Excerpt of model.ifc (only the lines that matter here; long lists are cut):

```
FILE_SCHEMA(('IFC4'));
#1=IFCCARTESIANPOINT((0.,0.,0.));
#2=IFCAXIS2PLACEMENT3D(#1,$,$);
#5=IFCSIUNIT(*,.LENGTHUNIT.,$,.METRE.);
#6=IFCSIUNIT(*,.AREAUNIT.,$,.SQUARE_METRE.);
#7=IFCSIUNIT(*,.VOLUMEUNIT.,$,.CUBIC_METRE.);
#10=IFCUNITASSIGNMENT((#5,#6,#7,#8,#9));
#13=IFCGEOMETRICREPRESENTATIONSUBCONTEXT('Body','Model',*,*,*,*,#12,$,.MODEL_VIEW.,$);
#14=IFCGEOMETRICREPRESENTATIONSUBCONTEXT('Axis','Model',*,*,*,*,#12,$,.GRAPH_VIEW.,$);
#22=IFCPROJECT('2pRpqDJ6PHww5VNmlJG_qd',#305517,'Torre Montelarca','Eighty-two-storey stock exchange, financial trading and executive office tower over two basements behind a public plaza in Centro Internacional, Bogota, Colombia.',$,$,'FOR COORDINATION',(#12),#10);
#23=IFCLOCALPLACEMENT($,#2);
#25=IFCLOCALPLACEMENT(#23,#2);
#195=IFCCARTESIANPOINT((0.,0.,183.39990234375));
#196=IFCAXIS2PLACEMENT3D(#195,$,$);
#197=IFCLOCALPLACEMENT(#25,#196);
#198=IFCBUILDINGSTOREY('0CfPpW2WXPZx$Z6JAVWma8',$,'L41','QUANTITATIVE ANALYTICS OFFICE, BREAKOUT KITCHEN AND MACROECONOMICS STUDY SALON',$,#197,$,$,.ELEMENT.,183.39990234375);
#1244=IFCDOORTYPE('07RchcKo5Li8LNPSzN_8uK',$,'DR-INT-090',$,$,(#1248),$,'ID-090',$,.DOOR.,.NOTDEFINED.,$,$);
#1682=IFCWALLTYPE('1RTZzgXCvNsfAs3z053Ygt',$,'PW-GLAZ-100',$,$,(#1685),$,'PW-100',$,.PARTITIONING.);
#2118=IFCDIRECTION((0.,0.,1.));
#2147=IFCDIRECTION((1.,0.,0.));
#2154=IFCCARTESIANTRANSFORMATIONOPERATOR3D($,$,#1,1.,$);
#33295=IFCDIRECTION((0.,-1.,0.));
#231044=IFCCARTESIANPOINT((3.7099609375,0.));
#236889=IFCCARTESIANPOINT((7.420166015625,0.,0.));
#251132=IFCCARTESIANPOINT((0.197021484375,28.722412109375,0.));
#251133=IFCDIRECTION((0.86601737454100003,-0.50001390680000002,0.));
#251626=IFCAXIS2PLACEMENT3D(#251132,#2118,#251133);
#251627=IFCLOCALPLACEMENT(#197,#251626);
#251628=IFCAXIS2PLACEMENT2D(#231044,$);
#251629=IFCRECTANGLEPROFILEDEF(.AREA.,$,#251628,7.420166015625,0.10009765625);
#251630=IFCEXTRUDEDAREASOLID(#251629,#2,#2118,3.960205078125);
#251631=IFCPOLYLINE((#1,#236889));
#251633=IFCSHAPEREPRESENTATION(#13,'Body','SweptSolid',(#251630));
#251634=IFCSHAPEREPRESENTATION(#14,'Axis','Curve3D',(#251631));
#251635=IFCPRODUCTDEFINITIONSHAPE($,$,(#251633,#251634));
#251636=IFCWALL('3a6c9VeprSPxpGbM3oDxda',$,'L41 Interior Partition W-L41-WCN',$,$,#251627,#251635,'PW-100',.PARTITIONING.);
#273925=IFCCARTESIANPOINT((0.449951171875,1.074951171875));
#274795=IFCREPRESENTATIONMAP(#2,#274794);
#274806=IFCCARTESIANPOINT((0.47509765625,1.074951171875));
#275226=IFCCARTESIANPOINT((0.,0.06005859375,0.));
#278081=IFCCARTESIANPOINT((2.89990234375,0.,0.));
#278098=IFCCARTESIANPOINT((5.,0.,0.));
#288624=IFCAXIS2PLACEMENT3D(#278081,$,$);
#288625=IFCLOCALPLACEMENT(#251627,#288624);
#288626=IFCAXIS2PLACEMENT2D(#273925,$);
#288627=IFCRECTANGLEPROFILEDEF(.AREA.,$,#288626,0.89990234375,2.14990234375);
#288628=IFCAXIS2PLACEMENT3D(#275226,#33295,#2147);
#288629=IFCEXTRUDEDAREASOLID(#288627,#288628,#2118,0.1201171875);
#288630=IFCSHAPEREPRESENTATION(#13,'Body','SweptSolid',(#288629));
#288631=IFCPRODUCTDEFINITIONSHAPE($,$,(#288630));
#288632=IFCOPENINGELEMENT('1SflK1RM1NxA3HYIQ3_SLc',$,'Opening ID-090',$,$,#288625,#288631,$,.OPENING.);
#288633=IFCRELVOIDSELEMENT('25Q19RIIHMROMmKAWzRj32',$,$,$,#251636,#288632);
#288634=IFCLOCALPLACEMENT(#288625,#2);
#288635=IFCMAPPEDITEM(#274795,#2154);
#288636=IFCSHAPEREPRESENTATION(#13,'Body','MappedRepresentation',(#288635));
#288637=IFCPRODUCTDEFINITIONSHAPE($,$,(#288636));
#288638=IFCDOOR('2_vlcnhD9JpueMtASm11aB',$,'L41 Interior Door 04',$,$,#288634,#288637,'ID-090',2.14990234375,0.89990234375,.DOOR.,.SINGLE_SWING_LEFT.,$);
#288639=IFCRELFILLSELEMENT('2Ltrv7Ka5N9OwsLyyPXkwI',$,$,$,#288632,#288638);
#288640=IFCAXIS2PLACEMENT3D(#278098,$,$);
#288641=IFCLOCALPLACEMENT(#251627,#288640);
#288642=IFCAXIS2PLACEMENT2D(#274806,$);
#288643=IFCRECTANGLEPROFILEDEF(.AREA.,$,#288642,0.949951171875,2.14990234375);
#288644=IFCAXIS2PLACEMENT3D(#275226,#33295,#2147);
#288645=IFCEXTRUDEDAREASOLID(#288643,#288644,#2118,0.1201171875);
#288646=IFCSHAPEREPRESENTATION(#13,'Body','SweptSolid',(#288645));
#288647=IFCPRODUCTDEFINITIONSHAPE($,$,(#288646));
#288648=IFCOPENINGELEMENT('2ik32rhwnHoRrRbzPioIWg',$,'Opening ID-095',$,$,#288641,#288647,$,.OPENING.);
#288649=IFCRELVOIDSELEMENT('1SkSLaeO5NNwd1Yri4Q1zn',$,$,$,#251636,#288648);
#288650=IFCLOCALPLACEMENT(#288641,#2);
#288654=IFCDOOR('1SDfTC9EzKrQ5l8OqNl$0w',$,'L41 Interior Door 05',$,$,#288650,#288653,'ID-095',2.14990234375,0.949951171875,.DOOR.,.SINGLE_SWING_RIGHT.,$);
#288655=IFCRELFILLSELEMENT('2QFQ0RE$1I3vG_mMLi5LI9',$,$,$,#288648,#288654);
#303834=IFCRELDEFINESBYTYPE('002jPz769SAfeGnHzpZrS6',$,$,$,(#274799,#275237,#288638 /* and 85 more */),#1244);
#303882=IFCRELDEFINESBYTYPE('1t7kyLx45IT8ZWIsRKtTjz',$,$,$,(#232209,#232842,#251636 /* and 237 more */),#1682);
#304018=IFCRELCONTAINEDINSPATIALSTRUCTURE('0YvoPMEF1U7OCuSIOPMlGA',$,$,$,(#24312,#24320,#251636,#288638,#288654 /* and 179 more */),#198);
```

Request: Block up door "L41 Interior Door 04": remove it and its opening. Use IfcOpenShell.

```python
import ifcopenshell
import ifcopenshell.api.feature
import ifcopenshell.api.root
import ifcopenshell.geom
import ifcopenshell.util.shape

model = ifcopenshell.open("model.ifc")
settings = ifcopenshell.geom.settings()


def volume(element):
    """Net volume in cubic metres, openings subtracted."""
    shape = ifcopenshell.geom.create_shape(settings, element)
    return ifcopenshell.util.shape.get_volume(shape.geometry)


door = model.by_guid("2_vlcnhD9JpueMtASm11aB")
opening = door.FillsVoids[0].RelatingOpeningElement
wall = opening.VoidsElements[0].RelatingBuildingElement
before = volume(wall)

ifcopenshell.api.root.remove_product(model, product=door)
ifcopenshell.api.feature.remove_feature(model, feature=opening)

after = volume(wall)

print(f"wall volume {before:.3f} -> {after:.3f} m3")

model.write("model-out.ifc")
```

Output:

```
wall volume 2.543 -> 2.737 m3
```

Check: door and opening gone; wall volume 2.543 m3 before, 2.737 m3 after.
